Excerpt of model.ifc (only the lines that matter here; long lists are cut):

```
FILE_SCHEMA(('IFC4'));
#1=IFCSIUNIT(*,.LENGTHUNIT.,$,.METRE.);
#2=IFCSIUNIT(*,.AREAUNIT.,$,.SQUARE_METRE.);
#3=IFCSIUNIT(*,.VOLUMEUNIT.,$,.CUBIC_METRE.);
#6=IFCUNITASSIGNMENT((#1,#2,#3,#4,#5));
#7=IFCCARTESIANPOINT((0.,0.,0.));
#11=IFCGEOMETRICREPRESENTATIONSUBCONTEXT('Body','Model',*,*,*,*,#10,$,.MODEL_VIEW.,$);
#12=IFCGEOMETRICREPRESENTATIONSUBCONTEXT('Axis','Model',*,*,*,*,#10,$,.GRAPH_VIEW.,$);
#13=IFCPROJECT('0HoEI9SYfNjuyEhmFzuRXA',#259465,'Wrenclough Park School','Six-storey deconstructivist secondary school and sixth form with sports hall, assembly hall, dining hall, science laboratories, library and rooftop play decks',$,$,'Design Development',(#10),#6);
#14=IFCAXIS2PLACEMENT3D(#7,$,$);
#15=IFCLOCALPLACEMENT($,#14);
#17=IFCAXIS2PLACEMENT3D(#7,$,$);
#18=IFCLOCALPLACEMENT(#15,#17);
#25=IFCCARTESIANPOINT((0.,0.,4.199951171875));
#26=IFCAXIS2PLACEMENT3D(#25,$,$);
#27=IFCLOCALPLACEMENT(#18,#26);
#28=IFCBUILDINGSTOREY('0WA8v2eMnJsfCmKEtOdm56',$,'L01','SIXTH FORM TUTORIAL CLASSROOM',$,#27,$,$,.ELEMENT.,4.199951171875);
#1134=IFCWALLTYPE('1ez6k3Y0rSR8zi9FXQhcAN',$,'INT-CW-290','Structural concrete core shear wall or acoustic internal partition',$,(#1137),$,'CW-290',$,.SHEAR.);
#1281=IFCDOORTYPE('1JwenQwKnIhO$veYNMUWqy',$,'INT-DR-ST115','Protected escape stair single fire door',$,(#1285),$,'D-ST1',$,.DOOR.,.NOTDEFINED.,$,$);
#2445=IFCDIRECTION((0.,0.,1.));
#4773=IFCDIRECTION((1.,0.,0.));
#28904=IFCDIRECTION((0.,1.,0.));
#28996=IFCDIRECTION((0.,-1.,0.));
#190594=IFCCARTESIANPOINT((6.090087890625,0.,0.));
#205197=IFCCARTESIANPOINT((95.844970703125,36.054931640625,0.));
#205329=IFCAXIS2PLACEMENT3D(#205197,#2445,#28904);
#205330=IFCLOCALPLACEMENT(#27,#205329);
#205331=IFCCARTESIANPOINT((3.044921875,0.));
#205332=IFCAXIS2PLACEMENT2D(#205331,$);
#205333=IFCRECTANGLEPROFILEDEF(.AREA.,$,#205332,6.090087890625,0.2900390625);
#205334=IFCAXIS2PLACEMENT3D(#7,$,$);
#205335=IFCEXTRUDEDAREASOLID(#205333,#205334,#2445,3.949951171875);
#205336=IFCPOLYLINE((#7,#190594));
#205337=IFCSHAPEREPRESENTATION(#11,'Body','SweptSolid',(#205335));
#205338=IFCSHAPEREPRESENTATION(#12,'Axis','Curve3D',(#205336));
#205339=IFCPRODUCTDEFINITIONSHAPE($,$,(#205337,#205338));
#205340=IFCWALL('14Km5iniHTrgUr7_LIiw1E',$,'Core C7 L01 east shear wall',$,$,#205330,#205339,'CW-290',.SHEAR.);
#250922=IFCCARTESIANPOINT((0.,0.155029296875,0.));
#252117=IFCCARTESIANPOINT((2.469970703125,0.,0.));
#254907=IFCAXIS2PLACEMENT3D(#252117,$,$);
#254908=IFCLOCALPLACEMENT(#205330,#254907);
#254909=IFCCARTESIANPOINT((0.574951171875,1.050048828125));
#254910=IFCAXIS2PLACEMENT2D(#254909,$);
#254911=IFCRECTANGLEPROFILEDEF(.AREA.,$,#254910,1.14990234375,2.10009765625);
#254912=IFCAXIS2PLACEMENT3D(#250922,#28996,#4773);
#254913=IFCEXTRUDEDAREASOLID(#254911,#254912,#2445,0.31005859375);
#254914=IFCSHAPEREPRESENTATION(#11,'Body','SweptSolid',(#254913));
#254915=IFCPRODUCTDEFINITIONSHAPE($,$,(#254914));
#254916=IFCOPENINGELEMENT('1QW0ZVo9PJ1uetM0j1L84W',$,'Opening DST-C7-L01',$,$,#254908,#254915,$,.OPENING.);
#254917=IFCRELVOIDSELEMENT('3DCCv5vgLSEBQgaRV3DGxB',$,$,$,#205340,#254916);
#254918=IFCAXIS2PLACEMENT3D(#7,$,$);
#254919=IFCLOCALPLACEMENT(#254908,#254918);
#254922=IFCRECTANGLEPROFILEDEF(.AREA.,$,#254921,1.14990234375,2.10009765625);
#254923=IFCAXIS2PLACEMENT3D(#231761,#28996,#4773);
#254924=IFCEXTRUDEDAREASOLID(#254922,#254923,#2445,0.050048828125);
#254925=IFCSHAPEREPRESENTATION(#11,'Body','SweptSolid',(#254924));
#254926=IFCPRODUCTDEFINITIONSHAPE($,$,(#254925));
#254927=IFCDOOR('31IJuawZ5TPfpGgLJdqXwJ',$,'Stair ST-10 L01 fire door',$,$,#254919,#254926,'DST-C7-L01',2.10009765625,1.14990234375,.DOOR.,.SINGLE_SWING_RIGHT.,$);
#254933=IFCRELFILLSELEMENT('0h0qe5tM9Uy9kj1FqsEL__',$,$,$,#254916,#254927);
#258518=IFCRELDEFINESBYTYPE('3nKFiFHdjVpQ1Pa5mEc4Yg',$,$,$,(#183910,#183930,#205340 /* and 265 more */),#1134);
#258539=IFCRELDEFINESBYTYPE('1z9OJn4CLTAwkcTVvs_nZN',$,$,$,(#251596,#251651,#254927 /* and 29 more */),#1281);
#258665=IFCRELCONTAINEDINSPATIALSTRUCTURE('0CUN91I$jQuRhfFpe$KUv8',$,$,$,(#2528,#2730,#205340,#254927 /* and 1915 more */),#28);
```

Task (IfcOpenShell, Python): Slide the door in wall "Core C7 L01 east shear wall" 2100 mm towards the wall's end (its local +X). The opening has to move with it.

```python
import ifcopenshell
import ifcopenshell.api.geometry
import ifcopenshell.util.placement
import ifcopenshell.util.unit

model = ifcopenshell.open("model.ifc")
unit_scale = ifcopenshell.util.unit.calculate_unit_scale(model)

door = model.by_guid("31IJuawZ5TPfpGgLJdqXwJ")
opening = door.FillsVoids[0].RelatingOpeningElement
wall = opening.VoidsElements[0].RelatingBuildingElement

wall_matrix = ifcopenshell.util.placement.get_local_placement(wall.ObjectPlacement)
shift = wall_matrix[:3, 0] * 2.1 / unit_scale
before = ifcopenshell.util.placement.get_local_placement(door.ObjectPlacement)[:3, 3].copy()

# The door is placed relative to its opening, so it follows when the opening moves.
matrix = ifcopenshell.util.placement.get_local_placement(opening.ObjectPlacement)
matrix[:3, 3] += shift
ifcopenshell.api.geometry.edit_object_placement(
    model, product=opening, matrix=matrix, is_si=False, should_transform_children=True
)

after = ifcopenshell.util.placement.get_local_placement(door.ObjectPlacement)[:3, 3]
print("door moved by", (after - before).round(3) + 0.0)

model.write("model_v2.ifc")
```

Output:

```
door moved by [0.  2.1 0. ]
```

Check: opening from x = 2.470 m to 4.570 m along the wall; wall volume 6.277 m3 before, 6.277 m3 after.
